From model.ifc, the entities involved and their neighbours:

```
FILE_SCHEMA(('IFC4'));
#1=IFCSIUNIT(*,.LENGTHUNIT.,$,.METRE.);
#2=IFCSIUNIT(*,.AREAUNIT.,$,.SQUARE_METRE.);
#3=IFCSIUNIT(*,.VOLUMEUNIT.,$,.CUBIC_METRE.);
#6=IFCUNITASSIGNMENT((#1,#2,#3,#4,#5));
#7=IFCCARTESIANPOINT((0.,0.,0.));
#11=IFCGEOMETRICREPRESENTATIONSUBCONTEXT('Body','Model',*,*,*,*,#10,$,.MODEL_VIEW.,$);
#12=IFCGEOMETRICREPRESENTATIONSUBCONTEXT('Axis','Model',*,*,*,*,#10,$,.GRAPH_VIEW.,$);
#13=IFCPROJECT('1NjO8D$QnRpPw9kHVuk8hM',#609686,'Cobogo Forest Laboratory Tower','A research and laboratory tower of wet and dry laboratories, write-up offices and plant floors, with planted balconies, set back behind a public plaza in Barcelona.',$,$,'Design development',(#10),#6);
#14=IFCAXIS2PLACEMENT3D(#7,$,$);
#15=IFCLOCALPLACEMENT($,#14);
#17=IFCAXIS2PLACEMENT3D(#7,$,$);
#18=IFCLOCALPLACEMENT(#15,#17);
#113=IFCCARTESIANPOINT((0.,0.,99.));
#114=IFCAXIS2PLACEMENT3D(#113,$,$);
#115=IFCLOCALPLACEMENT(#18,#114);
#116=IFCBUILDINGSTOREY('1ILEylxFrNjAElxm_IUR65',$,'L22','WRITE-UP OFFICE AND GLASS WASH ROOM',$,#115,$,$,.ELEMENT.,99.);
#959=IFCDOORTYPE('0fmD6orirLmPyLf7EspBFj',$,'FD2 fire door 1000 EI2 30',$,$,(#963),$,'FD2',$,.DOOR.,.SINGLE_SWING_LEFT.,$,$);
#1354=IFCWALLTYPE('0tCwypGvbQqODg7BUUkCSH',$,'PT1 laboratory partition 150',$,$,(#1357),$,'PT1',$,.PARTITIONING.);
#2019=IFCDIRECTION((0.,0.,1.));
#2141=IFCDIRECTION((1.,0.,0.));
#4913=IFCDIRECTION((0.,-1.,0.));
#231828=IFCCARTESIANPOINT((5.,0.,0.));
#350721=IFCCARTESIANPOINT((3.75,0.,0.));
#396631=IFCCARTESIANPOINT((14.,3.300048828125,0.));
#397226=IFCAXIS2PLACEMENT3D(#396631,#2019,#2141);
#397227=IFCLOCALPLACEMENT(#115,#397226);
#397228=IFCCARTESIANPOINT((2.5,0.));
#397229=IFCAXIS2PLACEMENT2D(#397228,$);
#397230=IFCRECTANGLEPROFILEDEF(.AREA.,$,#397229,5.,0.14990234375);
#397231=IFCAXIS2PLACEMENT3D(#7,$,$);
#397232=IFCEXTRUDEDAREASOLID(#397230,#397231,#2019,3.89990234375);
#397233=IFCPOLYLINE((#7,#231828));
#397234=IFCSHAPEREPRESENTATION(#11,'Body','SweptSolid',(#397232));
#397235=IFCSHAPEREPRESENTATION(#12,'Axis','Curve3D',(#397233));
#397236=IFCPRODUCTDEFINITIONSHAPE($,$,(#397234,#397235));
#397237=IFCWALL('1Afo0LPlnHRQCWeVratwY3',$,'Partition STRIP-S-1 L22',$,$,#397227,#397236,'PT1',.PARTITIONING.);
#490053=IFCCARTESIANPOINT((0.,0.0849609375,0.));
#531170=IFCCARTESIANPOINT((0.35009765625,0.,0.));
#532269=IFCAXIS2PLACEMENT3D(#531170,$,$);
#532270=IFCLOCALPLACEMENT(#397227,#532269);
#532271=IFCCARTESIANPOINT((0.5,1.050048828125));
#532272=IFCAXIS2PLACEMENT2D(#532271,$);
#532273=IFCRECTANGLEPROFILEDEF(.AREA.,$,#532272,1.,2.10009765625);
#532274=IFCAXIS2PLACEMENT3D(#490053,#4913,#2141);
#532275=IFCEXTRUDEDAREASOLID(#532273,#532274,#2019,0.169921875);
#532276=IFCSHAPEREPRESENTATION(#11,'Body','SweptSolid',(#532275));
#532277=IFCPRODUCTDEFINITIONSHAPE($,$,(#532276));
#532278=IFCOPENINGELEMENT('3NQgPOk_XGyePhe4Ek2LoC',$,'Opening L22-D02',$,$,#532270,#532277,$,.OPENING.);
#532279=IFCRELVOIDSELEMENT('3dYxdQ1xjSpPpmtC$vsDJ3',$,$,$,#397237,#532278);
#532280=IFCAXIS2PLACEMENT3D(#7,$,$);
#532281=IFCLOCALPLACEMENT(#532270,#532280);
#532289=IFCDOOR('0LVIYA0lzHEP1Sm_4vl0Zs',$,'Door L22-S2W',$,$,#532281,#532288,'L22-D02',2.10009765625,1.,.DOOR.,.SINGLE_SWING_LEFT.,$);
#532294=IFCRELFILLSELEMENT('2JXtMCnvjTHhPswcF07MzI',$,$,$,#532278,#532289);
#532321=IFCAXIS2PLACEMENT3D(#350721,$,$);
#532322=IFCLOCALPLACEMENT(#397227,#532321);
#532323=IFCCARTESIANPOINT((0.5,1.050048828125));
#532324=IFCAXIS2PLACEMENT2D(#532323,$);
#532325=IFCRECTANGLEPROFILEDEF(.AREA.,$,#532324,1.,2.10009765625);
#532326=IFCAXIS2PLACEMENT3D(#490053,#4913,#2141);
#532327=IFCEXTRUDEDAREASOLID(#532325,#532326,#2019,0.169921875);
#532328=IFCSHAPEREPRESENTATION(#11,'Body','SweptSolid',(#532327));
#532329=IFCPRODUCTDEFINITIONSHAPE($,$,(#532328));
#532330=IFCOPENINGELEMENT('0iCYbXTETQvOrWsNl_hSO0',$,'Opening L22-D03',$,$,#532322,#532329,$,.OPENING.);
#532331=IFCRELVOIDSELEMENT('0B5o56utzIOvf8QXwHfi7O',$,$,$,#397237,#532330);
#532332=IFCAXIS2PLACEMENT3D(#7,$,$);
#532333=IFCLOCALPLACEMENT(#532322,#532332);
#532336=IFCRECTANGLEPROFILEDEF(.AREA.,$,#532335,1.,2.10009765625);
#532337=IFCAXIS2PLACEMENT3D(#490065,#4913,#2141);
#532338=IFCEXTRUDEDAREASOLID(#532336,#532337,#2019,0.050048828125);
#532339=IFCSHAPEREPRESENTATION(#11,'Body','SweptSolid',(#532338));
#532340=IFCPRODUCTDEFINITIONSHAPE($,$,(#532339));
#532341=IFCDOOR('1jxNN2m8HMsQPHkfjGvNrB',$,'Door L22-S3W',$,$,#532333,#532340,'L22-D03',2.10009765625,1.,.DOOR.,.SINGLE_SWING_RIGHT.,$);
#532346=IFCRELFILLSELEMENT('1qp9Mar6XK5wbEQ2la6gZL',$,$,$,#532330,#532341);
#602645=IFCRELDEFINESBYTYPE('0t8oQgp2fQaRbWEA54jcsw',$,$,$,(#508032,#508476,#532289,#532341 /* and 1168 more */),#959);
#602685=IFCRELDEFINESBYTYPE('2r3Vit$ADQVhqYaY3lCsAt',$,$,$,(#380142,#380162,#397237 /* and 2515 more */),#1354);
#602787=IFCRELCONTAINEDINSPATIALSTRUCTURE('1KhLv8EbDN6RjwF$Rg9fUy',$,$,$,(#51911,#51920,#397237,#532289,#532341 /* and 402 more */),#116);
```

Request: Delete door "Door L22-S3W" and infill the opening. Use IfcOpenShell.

```python
import ifcopenshell
import ifcopenshell.api.feature
import ifcopenshell.api.root
import ifcopenshell.geom
import ifcopenshell.util.shape

model = ifcopenshell.open("model.ifc")
settings = ifcopenshell.geom.settings()


def volume(element):
    """Net volume in cubic metres, openings subtracted."""
    shape = ifcopenshell.geom.create_shape(settings, element)
    return ifcopenshell.util.shape.get_volume(shape.geometry)


door = model.by_guid("1jxNN2m8HMsQPHkfjGvNrB")
opening = door.FillsVoids[0].RelatingOpeningElement
wall = opening.VoidsElements[0].RelatingBuildingElement
before = volume(wall)

ifcopenshell.api.root.remove_product(model, product=door)
ifcopenshell.api.feature.remove_feature(model, feature=opening)

after = volume(wall)

print(f"wall volume {before:.3f} -> {after:.3f} m3")

model.write("model_updated.ifc")
```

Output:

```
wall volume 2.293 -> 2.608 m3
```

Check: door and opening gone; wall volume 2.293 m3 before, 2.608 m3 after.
